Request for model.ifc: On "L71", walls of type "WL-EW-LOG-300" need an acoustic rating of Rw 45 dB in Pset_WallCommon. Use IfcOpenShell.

First a look at what the model holds.

```python
import ifcopenshell
import ifcopenshell.util.element

model = ifcopenshell.open("model.ifc")
print(model.schema)
storey = next(s for s in model.by_type("IfcBuildingStorey") if s.Name == "L71")
walls = [e for e in ifcopenshell.util.element.get_decomposition(storey) if e.is_a("IfcWall")]
seen = {}
for e in walls:
    element_type = ifcopenshell.util.element.get_type(e)
    key = (element_type.Name if element_type != e and element_type else None, ifcopenshell.util.element.get_pset(e, "Pset_WallCommon", "AcousticRating"))
    seen[key] = seen.get(key, 0) + 1
for (name, value), count in sorted(seen.items(), key=str):
    print(count, "x", name, "|", value)
```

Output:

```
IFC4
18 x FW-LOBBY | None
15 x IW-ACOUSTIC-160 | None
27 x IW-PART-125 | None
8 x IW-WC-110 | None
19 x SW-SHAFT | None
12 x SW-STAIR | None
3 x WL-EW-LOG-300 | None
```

```python
import ifcopenshell
import ifcopenshell.api.pset
import ifcopenshell.util.element

model = ifcopenshell.open("model.ifc")

storey = next(s for s in model.by_type("IfcBuildingStorey") if s.Name == "L71")
walls = [e for e in ifcopenshell.util.element.get_decomposition(storey) if e.is_a("IfcWall")]

count = 0
for e in walls:
    element_type = ifcopenshell.util.element.get_type(e)
    if element_type in (None, e) or element_type.Name != "WL-EW-LOG-300":
        continue
    found = ifcopenshell.util.element.get_pset(e, "Pset_WallCommon", should_inherit=False)
    if found:
        pset = model.by_id(found["id"])
        if len(ifcopenshell.util.element.get_elements_by_pset(pset)) > 1:
            pset = ifcopenshell.api.pset.unshare_pset(model, products=[e], pset=pset)[0]
    else:
        pset = ifcopenshell.api.pset.add_pset(model, product=e, name="Pset_WallCommon")
    ifcopenshell.api.pset.edit_pset(model, pset=pset, properties={"AcousticRating": "Rw 45 dB"})
    count += 1

print(count, "walls updated")

model.write("model_updated.ifc")
```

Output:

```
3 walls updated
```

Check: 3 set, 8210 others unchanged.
